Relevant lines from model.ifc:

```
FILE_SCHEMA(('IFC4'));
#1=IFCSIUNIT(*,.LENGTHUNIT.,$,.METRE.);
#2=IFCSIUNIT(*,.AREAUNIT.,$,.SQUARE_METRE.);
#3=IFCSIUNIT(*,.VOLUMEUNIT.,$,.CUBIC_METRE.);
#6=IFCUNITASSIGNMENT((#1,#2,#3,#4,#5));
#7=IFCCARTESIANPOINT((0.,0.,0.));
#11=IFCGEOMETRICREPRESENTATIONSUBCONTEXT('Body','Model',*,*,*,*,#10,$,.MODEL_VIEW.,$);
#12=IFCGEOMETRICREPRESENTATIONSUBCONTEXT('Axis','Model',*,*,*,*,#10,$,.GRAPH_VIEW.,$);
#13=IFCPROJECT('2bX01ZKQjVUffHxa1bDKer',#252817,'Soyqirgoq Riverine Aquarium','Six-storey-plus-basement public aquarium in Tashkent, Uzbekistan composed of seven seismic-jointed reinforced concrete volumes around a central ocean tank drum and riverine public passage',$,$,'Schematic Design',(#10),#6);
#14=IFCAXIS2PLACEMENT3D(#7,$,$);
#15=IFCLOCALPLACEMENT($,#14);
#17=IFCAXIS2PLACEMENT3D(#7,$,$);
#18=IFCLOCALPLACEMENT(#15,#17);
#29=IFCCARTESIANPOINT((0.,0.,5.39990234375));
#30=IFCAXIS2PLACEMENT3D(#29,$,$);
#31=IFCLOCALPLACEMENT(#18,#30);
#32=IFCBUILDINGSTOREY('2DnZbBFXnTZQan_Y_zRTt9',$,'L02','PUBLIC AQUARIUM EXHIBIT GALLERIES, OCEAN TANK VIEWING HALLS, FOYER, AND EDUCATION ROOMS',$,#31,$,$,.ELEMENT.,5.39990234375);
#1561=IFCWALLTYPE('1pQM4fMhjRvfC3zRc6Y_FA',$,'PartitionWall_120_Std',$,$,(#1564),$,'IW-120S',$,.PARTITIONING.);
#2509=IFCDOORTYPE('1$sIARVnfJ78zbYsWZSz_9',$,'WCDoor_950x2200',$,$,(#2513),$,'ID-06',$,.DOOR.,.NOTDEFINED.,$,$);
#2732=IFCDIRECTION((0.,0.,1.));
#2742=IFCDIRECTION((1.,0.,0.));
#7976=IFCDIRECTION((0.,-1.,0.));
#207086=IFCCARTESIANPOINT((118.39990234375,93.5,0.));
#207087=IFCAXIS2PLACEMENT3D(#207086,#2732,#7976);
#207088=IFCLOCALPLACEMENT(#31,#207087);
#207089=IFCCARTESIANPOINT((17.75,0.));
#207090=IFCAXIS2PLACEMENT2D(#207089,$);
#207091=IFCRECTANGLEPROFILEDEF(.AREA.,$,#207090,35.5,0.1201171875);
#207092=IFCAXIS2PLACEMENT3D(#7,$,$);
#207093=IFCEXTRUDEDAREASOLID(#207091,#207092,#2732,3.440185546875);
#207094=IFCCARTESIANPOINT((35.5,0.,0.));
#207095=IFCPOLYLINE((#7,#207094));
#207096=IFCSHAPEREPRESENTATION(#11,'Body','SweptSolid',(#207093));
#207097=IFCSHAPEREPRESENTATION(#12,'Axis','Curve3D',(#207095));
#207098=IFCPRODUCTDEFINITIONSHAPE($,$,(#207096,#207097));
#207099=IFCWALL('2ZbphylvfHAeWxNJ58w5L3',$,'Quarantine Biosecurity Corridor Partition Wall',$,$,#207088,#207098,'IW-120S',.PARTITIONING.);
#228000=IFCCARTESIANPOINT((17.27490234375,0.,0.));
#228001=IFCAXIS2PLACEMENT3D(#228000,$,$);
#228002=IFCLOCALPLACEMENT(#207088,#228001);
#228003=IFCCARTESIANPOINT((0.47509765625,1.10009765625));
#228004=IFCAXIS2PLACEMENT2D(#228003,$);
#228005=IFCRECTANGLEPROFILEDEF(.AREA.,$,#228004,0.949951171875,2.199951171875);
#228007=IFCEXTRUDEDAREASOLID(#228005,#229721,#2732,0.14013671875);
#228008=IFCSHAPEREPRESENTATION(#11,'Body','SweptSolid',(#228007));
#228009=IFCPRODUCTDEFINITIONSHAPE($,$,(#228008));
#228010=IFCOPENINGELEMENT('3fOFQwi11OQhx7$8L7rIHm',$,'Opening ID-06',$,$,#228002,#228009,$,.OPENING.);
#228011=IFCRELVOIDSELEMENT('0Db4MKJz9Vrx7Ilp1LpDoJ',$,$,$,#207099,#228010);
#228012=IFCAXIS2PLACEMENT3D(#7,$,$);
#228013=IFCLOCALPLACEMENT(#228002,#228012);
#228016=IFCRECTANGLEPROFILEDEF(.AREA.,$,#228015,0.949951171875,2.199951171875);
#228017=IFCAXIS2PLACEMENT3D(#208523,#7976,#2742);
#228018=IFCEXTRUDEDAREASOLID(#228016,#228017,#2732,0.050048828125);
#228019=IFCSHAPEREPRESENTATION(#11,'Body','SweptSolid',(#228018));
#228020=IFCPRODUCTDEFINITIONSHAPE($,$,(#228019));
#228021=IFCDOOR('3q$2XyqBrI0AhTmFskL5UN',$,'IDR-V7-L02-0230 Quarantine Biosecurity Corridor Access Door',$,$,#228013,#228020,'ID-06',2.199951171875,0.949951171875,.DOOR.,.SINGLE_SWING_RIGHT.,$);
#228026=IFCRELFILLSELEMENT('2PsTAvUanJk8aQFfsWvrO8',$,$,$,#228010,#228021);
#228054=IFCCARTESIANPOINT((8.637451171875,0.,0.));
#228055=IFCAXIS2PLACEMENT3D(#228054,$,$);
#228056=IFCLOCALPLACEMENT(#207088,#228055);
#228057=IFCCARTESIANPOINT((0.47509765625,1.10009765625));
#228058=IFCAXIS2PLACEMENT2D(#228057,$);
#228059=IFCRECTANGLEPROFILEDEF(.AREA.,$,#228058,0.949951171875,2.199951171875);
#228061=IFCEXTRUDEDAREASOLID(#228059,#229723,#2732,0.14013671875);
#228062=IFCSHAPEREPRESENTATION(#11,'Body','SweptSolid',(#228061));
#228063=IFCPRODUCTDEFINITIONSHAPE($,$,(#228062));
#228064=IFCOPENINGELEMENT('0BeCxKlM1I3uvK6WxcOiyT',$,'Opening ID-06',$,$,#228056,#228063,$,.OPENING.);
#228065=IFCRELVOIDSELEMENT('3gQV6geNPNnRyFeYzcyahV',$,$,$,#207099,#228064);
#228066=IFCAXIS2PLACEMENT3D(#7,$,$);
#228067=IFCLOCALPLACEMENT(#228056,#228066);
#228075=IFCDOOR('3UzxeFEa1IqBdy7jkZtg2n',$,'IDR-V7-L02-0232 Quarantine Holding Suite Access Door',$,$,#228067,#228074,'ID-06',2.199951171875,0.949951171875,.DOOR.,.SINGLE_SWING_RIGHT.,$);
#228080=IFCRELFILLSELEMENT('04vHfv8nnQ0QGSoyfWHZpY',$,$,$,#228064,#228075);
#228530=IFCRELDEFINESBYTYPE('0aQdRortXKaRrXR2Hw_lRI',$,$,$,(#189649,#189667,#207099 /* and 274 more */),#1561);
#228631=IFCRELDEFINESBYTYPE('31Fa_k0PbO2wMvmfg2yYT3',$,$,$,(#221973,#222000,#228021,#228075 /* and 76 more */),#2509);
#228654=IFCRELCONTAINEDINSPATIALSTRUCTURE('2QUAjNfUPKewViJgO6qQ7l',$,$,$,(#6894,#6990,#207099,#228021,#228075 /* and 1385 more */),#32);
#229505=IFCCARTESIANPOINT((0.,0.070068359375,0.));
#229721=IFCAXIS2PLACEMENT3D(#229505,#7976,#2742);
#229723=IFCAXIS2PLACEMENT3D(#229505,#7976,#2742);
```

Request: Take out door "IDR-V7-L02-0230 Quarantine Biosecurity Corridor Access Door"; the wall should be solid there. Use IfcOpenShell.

```python
import ifcopenshell
import ifcopenshell.api.feature
import ifcopenshell.api.root
import ifcopenshell.geom
import ifcopenshell.util.shape

model = ifcopenshell.open("model.ifc")
settings = ifcopenshell.geom.settings()


def volume(element):
    """Net volume in cubic metres, openings subtracted."""
    shape = ifcopenshell.geom.create_shape(settings, element)
    return ifcopenshell.util.shape.get_volume(shape.geometry)


door = model.by_guid("3q$2XyqBrI0AhTmFskL5UN")
opening = door.FillsVoids[0].RelatingOpeningElement
wall = opening.VoidsElements[0].RelatingBuildingElement
before = volume(wall)

ifcopenshell.api.root.remove_product(model, product=door)
ifcopenshell.api.feature.remove_feature(model, feature=opening)

after = volume(wall)

print(f"wall volume {before:.3f} -> {after:.3f} m3")

model.write("model_edited.ifc")
```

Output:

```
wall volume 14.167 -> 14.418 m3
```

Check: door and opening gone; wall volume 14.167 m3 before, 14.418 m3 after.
